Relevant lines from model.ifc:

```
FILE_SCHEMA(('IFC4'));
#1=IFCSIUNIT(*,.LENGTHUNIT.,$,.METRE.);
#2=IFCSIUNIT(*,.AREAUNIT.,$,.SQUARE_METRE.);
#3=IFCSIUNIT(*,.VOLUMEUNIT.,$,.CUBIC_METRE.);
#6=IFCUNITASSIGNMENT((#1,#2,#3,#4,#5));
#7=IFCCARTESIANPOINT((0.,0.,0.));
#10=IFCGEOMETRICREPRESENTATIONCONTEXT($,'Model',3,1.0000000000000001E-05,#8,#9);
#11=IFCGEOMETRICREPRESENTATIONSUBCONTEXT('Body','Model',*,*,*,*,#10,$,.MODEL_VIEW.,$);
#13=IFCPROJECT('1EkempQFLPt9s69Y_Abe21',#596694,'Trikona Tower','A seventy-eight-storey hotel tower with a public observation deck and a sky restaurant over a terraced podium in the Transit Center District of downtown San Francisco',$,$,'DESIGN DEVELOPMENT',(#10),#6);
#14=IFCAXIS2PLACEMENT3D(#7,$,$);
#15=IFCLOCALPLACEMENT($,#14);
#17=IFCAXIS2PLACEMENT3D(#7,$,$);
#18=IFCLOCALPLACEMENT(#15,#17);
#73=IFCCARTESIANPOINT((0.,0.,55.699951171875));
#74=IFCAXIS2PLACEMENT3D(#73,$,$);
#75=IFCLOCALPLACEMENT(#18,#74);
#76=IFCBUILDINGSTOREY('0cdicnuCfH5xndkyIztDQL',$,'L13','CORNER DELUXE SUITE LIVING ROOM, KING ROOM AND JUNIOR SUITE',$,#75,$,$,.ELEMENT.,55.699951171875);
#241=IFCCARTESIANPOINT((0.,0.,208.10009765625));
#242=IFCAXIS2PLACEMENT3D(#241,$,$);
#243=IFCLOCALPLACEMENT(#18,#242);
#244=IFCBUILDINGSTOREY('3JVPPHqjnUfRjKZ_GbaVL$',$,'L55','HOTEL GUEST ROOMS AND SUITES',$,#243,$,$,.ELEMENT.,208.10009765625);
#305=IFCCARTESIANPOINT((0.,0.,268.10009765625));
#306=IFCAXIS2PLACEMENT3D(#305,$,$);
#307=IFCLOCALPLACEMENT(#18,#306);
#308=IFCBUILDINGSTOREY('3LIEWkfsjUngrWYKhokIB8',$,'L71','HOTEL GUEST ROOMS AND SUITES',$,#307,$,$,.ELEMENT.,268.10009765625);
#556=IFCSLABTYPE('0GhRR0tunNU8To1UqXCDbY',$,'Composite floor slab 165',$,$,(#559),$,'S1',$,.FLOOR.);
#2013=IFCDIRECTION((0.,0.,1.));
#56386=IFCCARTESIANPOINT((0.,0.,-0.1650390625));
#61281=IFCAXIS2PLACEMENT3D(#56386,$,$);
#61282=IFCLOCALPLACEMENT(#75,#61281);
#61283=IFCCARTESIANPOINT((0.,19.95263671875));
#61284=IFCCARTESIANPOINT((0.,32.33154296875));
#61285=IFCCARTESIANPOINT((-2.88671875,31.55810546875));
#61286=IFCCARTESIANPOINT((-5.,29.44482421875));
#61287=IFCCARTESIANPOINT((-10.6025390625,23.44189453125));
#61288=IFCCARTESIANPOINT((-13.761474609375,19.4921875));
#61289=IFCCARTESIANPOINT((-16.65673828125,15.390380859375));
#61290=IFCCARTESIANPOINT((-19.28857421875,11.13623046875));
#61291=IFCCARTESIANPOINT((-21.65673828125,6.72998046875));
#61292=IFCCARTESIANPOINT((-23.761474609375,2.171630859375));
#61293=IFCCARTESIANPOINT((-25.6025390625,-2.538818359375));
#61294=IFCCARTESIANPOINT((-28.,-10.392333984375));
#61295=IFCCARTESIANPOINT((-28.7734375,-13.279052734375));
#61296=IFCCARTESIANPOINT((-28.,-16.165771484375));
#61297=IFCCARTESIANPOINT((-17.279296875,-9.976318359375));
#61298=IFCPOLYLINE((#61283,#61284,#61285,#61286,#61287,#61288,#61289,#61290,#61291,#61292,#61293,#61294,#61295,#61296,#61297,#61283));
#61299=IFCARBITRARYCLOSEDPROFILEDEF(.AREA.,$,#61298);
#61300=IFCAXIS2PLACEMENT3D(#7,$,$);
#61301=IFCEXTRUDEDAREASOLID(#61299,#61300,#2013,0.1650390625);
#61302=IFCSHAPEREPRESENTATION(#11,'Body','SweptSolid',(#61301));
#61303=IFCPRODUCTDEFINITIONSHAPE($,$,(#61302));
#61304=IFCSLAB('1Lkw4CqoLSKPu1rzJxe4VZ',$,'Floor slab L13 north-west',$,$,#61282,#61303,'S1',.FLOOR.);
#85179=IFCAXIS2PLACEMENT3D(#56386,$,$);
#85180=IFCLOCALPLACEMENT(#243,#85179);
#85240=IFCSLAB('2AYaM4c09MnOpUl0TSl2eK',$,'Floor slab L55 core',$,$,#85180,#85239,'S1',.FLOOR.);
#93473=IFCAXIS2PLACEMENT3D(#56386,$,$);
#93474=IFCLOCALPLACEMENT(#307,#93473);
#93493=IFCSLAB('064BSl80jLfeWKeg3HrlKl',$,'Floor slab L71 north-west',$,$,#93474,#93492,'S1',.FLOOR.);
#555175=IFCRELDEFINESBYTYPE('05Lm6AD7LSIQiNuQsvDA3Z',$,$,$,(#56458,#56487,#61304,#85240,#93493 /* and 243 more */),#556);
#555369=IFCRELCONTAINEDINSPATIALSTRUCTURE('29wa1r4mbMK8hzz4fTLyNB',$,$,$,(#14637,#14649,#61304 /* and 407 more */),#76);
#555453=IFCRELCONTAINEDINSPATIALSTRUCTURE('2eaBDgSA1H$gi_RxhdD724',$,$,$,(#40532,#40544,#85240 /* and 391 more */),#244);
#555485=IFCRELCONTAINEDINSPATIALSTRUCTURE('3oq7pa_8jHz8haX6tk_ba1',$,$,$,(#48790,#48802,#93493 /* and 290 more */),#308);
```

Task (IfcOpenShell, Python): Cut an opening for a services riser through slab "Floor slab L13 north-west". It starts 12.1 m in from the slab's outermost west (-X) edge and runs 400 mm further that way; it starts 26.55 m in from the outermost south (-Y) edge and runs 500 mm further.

```python
import numpy as np
import ifcopenshell
import ifcopenshell.api.feature
import ifcopenshell.api.geometry
import ifcopenshell.api.root
import ifcopenshell.geom
import ifcopenshell.util.placement
import ifcopenshell.util.representation
import ifcopenshell.util.shape
import ifcopenshell.util.unit

model = ifcopenshell.open("model.ifc")
unit_scale = ifcopenshell.util.unit.calculate_unit_scale(model)
settings = ifcopenshell.geom.settings()


def volume(element):
    """Net volume in cubic metres, openings subtracted."""
    shape = ifcopenshell.geom.create_shape(settings, element)
    return ifcopenshell.util.shape.get_volume(shape.geometry)


slab = model.by_guid("1Lkw4CqoLSKPu1rzJxe4VZ")
before = volume(slab)

# Extent in the slab's own axes, in metres. The edges named are its -X and -Y sides.
slab_shape = ifcopenshell.geom.create_shape(settings, slab)
vertices = ifcopenshell.util.shape.get_vertices(slab_shape.geometry)
x_min, y_min, bottom = vertices.min(axis=0)
top = vertices[:, 2].max()

opening = ifcopenshell.api.root.create_entity(model, ifc_class="IfcOpeningElement", name="Services riser opening", predefined_type="OPENING")
context = ifcopenshell.util.representation.get_context(model, "Model", "Body", "MODEL_VIEW")
width, depth = 0.4, 0.5
outline = [(0.0, 0.0), (width, 0.0), (width, depth), (0.0, depth), (0.0, 0.0)]
# Overshoot both faces by 50 mm so the cut is clean.
shape = ifcopenshell.api.geometry.add_slab_representation(
    model, context=context, depth=top - bottom + 0.1, polyline=outline
)
ifcopenshell.api.geometry.assign_representation(model, product=opening, representation=shape)

matrix = ifcopenshell.util.placement.get_local_placement(slab.ObjectPlacement)
matrix[:, 3] = matrix @ np.append(np.array([x_min + 12.1, y_min + 26.55, bottom - 0.05]) / unit_scale, 1.0)
ifcopenshell.api.geometry.edit_object_placement(model, product=opening, matrix=matrix, is_si=False)
ifcopenshell.api.feature.add_feature(model, feature=opening, element=slab)

after = volume(slab)

print(f"slab volume {before:.3f} -> {after:.3f} m3")

model.write("model_updated.ifc")
```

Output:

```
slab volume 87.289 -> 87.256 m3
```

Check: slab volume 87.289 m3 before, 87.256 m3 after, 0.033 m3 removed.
